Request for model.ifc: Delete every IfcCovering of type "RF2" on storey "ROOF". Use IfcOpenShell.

First a look at what the model holds.

```python
import ifcopenshell
import ifcopenshell.util.element

model = ifcopenshell.open("model.ifc")
print(model.schema)
storey = next(s for s in model.by_type("IfcBuildingStorey") if s.Name == "ROOF")
coverings = [e for e in ifcopenshell.util.element.get_decomposition(storey) if e.is_a("IfcCovering")]
seen = {}
for e in coverings:
    element_type = ifcopenshell.util.element.get_type(e)
    name = element_type.Name if element_type not in (None, e) else None
    seen[name] = seen.get(name, 0) + 1
for name, count in sorted(seen.items(), key=str):
    print(count, "x", name)
```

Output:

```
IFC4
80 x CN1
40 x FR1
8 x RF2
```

```python
import ifcopenshell
import ifcopenshell.api.root
import ifcopenshell.util.element

model = ifcopenshell.open("model.ifc")

storey = next(s for s in model.by_type("IfcBuildingStorey") if s.Name == "ROOF")
coverings = [e for e in ifcopenshell.util.element.get_decomposition(storey) if e.is_a("IfcCovering")]
targets = [e for e in coverings if (t := ifcopenshell.util.element.get_type(e)) not in (None, e) and t.Name == "RF2"]

for e in targets:
    ifcopenshell.api.root.remove_product(model, product=e)
print(len(targets), "removed")

model.write("model_v2.ifc")
```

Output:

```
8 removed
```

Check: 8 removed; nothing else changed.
